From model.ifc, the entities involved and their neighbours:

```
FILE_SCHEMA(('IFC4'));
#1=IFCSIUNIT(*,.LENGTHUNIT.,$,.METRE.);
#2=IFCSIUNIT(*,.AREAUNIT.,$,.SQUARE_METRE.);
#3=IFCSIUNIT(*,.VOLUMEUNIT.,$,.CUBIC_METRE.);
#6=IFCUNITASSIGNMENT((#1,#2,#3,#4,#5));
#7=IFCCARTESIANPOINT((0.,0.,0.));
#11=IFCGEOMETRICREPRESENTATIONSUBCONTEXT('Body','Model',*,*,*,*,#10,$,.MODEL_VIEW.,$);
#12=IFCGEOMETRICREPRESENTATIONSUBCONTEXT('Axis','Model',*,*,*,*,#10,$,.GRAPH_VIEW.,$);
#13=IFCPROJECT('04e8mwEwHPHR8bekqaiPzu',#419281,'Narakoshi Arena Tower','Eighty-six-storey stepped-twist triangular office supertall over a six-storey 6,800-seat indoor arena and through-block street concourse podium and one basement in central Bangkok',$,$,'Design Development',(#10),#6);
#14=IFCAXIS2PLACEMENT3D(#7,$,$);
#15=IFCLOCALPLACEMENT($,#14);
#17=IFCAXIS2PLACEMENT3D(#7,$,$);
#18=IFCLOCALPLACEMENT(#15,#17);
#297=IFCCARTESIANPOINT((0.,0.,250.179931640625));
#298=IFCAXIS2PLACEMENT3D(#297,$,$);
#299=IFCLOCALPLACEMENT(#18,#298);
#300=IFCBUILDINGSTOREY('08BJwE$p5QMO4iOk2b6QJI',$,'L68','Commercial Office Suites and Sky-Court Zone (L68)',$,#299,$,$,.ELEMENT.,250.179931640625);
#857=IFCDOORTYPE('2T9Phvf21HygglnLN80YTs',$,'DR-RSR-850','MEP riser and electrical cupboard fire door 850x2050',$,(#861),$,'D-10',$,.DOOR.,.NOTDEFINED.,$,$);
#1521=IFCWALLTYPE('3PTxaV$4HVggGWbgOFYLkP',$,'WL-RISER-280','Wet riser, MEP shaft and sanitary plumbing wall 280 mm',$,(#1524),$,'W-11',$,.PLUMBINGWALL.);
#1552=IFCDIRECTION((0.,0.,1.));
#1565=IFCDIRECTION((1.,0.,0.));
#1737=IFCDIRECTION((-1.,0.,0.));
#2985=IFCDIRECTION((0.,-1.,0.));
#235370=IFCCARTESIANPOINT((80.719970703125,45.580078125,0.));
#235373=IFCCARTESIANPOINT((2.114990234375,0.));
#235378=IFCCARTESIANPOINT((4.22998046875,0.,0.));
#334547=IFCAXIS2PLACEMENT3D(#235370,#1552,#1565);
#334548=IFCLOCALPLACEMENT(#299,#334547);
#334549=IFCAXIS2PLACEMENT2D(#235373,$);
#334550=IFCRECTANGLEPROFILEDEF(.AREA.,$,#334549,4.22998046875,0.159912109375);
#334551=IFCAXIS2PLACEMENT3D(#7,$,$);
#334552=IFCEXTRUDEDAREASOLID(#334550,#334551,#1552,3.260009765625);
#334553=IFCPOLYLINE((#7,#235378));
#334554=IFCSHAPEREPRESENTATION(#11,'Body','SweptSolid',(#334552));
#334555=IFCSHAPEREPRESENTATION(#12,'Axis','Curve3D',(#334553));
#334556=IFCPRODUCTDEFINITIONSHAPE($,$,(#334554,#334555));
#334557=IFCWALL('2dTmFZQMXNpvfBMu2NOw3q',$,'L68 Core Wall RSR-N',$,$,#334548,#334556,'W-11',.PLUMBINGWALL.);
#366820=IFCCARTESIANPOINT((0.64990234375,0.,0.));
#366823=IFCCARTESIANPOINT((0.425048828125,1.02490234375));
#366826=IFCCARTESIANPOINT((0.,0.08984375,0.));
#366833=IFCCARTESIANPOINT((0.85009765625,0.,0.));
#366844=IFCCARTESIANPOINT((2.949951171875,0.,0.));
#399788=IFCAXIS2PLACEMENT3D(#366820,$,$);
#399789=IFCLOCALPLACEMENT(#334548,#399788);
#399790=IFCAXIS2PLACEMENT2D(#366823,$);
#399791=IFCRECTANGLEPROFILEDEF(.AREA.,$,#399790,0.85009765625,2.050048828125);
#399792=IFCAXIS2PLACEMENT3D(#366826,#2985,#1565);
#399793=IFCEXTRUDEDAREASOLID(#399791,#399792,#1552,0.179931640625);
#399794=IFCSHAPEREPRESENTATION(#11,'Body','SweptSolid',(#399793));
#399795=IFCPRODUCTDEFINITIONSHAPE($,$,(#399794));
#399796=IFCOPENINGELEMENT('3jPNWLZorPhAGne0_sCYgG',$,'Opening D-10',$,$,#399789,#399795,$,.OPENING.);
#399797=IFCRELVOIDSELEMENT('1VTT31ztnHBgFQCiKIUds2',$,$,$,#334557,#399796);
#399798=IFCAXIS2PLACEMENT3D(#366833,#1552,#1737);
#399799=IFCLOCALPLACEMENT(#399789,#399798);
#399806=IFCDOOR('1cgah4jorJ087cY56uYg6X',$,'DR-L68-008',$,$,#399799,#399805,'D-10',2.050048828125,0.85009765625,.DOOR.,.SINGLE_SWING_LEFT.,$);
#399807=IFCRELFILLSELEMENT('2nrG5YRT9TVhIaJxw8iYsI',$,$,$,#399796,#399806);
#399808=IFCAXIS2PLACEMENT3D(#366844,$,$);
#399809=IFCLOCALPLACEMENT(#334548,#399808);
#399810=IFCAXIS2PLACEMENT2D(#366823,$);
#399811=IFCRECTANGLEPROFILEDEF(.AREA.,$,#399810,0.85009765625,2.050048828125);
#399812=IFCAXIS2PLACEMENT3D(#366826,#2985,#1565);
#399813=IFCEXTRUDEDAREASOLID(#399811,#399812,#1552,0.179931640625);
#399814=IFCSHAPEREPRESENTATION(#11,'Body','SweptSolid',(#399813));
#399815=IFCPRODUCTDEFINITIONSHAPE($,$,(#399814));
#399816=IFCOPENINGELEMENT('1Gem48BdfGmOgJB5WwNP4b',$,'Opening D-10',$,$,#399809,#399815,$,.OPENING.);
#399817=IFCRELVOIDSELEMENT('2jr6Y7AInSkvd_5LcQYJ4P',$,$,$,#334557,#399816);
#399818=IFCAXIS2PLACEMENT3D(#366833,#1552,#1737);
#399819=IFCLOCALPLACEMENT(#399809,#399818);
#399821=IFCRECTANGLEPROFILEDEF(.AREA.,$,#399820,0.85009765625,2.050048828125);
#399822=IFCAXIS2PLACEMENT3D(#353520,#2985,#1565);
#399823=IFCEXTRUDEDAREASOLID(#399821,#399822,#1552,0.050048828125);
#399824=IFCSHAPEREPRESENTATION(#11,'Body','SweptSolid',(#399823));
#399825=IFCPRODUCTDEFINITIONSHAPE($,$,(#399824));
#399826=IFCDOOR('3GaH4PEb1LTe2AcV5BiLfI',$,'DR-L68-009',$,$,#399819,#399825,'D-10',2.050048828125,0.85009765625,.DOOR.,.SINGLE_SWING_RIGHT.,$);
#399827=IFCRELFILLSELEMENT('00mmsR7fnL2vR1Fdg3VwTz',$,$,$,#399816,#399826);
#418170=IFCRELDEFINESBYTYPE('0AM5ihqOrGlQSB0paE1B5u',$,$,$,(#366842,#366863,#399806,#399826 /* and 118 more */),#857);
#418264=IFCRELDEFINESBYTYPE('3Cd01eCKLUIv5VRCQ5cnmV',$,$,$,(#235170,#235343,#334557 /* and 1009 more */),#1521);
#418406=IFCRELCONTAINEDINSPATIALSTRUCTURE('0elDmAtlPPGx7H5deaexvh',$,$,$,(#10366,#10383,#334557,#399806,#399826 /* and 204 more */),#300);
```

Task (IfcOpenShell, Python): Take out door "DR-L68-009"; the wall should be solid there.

```python
import ifcopenshell
import ifcopenshell.api.feature
import ifcopenshell.api.root
import ifcopenshell.geom
import ifcopenshell.util.shape

model = ifcopenshell.open("model.ifc")
settings = ifcopenshell.geom.settings()


def volume(element):
    """Net volume in cubic metres, openings subtracted."""
    shape = ifcopenshell.geom.create_shape(settings, element)
    return ifcopenshell.util.shape.get_volume(shape.geometry)


door = model.by_guid("3GaH4PEb1LTe2AcV5BiLfI")
opening = door.FillsVoids[0].RelatingOpeningElement
wall = opening.VoidsElements[0].RelatingBuildingElement
before = volume(wall)

ifcopenshell.api.root.remove_product(model, product=door)
ifcopenshell.api.feature.remove_feature(model, feature=opening)

after = volume(wall)

print(f"wall volume {before:.3f} -> {after:.3f} m3")

model.write("model_updated.ifc")
```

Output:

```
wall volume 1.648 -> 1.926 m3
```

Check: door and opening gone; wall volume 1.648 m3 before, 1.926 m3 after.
